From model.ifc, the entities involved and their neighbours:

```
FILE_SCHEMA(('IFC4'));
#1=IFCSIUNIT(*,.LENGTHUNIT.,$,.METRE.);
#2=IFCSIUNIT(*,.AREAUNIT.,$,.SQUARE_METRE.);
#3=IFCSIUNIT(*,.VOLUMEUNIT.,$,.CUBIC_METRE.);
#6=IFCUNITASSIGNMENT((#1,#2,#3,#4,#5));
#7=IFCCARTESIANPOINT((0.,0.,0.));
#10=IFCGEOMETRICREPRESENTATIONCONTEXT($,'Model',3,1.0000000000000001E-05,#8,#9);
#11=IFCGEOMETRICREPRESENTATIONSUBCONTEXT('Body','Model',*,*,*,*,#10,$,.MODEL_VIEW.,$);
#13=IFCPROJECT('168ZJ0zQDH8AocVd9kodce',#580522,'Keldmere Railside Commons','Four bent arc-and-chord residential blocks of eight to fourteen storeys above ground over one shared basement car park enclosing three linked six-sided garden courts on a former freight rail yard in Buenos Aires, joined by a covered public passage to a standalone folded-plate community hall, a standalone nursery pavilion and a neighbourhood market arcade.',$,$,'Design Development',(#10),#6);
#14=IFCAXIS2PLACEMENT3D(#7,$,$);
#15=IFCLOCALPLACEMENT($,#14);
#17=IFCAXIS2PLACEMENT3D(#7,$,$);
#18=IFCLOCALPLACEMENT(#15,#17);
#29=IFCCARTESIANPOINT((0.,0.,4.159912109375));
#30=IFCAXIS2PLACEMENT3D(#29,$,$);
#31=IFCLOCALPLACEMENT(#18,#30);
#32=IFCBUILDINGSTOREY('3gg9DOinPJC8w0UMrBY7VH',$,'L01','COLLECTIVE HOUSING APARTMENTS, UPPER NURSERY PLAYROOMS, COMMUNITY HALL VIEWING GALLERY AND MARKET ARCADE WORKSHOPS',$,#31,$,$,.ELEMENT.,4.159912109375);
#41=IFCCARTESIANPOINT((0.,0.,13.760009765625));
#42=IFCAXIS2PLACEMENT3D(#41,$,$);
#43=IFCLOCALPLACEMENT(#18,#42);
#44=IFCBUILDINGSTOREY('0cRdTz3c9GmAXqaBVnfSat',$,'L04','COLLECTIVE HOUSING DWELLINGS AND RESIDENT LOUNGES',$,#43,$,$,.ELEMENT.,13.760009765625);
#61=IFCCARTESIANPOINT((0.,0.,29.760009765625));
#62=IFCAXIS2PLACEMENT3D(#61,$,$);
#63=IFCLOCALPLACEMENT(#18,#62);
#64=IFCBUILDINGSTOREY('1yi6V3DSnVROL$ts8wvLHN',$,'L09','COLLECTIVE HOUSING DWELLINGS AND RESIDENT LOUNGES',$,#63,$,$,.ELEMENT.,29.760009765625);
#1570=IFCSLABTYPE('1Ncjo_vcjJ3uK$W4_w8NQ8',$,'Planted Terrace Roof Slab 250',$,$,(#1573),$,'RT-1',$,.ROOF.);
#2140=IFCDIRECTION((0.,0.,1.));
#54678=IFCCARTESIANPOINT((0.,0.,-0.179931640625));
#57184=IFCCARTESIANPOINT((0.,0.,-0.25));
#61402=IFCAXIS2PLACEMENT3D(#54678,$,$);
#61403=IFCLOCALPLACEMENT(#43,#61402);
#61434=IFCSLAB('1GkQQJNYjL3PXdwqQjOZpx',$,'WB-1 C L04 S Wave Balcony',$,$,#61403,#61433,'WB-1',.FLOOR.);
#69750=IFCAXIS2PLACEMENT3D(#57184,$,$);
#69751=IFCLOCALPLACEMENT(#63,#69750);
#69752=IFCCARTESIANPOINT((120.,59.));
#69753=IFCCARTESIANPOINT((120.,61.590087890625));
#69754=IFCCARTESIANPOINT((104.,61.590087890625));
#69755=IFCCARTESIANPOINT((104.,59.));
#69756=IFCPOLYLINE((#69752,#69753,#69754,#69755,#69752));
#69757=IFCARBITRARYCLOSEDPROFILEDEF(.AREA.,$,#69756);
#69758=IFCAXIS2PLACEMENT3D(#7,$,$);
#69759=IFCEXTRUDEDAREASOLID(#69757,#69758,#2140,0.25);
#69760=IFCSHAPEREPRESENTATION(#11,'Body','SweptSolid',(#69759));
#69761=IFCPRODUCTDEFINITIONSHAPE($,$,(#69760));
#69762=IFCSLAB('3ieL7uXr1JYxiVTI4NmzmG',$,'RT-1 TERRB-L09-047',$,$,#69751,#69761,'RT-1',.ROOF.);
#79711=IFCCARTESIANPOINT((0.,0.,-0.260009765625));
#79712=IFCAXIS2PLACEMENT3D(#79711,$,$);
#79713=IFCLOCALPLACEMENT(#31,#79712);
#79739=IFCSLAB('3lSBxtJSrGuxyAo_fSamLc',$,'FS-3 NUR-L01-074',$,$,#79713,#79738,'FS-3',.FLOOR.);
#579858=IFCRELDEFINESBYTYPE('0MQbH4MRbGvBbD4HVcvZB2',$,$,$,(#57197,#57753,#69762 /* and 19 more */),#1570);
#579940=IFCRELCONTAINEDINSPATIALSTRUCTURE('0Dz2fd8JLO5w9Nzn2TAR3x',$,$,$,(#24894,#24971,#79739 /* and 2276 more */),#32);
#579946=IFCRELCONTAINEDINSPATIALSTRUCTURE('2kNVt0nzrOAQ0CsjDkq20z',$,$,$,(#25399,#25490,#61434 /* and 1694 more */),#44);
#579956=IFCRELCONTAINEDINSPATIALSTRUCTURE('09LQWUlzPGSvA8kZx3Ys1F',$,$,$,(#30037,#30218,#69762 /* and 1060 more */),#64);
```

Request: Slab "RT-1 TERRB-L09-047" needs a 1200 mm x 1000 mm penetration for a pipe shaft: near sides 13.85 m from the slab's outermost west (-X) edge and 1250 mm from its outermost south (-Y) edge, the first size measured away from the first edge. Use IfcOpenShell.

```python
import numpy as np
import ifcopenshell
import ifcopenshell.api.feature
import ifcopenshell.api.geometry
import ifcopenshell.api.root
import ifcopenshell.geom
import ifcopenshell.util.placement
import ifcopenshell.util.representation
import ifcopenshell.util.shape
import ifcopenshell.util.unit

model = ifcopenshell.open("model.ifc")
unit_scale = ifcopenshell.util.unit.calculate_unit_scale(model)
settings = ifcopenshell.geom.settings()


def volume(element):
    """Net volume in cubic metres, openings subtracted."""
    shape = ifcopenshell.geom.create_shape(settings, element)
    return ifcopenshell.util.shape.get_volume(shape.geometry)


slab = model.by_guid("3ieL7uXr1JYxiVTI4NmzmG")
before = volume(slab)

# Extent in the slab's own axes, in metres. The edges named are its -X and -Y sides.
slab_shape = ifcopenshell.geom.create_shape(settings, slab)
vertices = ifcopenshell.util.shape.get_vertices(slab_shape.geometry)
x_min, y_min, bottom = vertices.min(axis=0)
top = vertices[:, 2].max()

opening = ifcopenshell.api.root.create_entity(model, ifc_class="IfcOpeningElement", name="Pipe shaft opening", predefined_type="OPENING")
context = ifcopenshell.util.representation.get_context(model, "Model", "Body", "MODEL_VIEW")
width, depth = 1.2, 1
outline = [(0.0, 0.0), (width, 0.0), (width, depth), (0.0, depth), (0.0, 0.0)]
# Overshoot both faces by 50 mm so the cut is clean.
shape = ifcopenshell.api.geometry.add_slab_representation(
    model, context=context, depth=top - bottom + 0.1, polyline=outline
)
ifcopenshell.api.geometry.assign_representation(model, product=opening, representation=shape)

matrix = ifcopenshell.util.placement.get_local_placement(slab.ObjectPlacement)
matrix[:, 3] = matrix @ np.append(np.array([x_min + 13.85, y_min + 1.25, bottom - 0.05]) / unit_scale, 1.0)
ifcopenshell.api.geometry.edit_object_placement(model, product=opening, matrix=matrix, is_si=False)
ifcopenshell.api.feature.add_feature(model, feature=opening, element=slab)

after = volume(slab)

print(f"slab volume {before:.3f} -> {after:.3f} m3")

model.write("model_v2.ifc")
```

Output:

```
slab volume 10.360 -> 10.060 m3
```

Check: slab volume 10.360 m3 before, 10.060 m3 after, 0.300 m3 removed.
